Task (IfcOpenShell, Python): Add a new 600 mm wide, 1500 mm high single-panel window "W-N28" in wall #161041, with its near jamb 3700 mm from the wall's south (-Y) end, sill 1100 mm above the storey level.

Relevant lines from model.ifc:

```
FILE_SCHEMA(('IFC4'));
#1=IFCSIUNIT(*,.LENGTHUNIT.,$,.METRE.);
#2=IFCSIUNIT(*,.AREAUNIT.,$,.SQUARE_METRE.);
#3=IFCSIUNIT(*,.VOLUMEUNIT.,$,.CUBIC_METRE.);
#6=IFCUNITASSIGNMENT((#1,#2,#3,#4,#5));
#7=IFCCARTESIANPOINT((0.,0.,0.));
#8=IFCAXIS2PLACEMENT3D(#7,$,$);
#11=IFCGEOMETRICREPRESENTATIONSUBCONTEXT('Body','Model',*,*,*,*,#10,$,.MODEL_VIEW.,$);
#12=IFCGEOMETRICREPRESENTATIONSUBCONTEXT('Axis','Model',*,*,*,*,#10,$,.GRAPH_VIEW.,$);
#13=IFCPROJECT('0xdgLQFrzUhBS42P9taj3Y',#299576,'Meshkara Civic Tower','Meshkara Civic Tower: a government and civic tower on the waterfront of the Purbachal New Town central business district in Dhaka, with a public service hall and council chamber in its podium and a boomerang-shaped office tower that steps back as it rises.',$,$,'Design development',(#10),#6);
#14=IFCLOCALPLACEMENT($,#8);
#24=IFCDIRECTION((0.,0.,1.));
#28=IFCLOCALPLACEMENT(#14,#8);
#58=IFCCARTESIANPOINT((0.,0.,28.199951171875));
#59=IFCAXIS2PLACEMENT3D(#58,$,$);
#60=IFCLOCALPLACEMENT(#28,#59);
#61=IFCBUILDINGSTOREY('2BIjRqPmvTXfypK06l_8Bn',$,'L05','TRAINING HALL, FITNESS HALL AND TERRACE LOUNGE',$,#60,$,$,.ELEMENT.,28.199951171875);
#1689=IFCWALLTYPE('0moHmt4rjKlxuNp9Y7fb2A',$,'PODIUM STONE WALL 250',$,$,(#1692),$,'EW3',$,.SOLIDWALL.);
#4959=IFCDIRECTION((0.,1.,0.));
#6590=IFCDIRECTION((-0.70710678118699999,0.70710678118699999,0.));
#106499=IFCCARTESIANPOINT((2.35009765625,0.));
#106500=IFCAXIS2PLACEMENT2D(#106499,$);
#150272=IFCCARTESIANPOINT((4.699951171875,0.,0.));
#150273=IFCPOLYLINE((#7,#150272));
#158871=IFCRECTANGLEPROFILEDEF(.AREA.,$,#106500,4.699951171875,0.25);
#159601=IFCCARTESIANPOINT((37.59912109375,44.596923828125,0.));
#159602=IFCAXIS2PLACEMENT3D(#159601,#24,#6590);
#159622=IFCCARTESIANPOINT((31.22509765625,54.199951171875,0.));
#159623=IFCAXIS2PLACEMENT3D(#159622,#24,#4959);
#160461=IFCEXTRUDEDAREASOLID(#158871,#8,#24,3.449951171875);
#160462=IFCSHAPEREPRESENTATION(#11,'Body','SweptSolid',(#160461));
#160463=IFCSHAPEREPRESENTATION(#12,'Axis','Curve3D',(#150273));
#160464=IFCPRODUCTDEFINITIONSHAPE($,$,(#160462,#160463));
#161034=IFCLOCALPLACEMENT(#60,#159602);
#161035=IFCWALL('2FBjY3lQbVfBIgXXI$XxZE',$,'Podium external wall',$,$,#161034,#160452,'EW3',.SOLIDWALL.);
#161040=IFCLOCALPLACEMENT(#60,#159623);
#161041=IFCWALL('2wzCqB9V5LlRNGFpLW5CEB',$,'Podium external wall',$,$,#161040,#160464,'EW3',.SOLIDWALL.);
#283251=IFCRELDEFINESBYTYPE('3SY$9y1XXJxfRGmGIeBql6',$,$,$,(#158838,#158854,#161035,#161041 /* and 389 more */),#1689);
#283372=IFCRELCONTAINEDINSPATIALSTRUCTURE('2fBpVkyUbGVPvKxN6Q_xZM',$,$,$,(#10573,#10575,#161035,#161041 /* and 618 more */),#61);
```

```python
import numpy as np
import ifcopenshell
import ifcopenshell.api.feature
import ifcopenshell.api.geometry
import ifcopenshell.api.root
import ifcopenshell.api.spatial
import ifcopenshell.geom
import ifcopenshell.util.element
import ifcopenshell.util.placement
import ifcopenshell.util.representation
import ifcopenshell.util.shape
import ifcopenshell.util.unit

model = ifcopenshell.open("model.ifc")
unit_scale = ifcopenshell.util.unit.calculate_unit_scale(model)
settings = ifcopenshell.geom.settings()


def volume(element):
    """Net volume in cubic metres, openings subtracted."""
    shape = ifcopenshell.geom.create_shape(settings, element)
    return ifcopenshell.util.shape.get_volume(shape.geometry)


wall = model.by_guid("2wzCqB9V5LlRNGFpLW5CEB")
storey = ifcopenshell.util.element.get_container(wall, ifc_class="IfcBuildingStorey")
context = ifcopenshell.util.representation.get_context(model, "Model", "Body", "MODEL_VIEW")
before = volume(wall)

width, height, from_end, sill = 0.6, 1.5, 3.7, 1.1  # metres

# The wall runs along its own X axis, and the end named is its -X end.
wall_shape = ifcopenshell.geom.create_shape(settings, wall)
x, y, z = ifcopenshell.util.shape.get_vertices(wall_shape.geometry).T
start = x.min() + from_end
face, thickness = float(y.min()), float(y.max() - y.min())
wall_matrix = ifcopenshell.util.placement.get_local_placement(wall.ObjectPlacement)
level = ifcopenshell.util.placement.get_local_placement(storey.ObjectPlacement)[2, 3]


def in_wall(x, y):
    """Placement at x, y metres in the wall's axes, at sill height."""
    matrix = wall_matrix.copy()
    matrix[:, 3] = wall_matrix @ np.array([x / unit_scale, y / unit_scale, 0.0, 1.0])
    matrix[2, 3] = level + sill / unit_scale
    return matrix


# Opening: a box that overshoots both wall faces by 50 mm.
opening = ifcopenshell.api.root.create_entity(model, ifc_class="IfcOpeningElement", predefined_type="OPENING")
box = ifcopenshell.api.geometry.add_wall_representation(
    model, context=context, length=width, height=height, thickness=thickness + 0.1
)
ifcopenshell.api.geometry.assign_representation(model, product=opening, representation=box)
ifcopenshell.api.geometry.edit_object_placement(model, product=opening, matrix=in_wall(start, face - 0.05), is_si=False)
ifcopenshell.api.feature.add_feature(model, feature=opening, element=wall)

window = ifcopenshell.api.root.create_entity(model, ifc_class="IfcWindow", name="W-N28", predefined_type="WINDOW")
window.OverallWidth, window.OverallHeight = width / unit_scale, height / unit_scale
window.PartitioningType = "SINGLE_PANEL"
body = ifcopenshell.api.geometry.add_window_representation(
    model,
    context=context,
    overall_width=window.OverallWidth,
    overall_height=window.OverallHeight,
    partition_type="SINGLE_PANEL",
)
ifcopenshell.api.geometry.assign_representation(model, product=window, representation=body)
ifcopenshell.api.spatial.assign_container(model, products=[window], relating_structure=storey)
ifcopenshell.api.feature.add_filling(model, opening=opening, element=window)

# Centre the window in the wall's thickness.
ifcopenshell.api.geometry.edit_object_placement(model, product=window, matrix=in_wall(start, face), is_si=False)
window_shape = ifcopenshell.geom.create_shape(settings, window)
depth = ifcopenshell.util.shape.get_vertices(window_shape.geometry)[:, 1]
offset = face + thickness / 2 - (depth.min() + depth.max()) / 2
ifcopenshell.api.geometry.edit_object_placement(model, product=window, matrix=in_wall(start, offset), is_si=False)

after = volume(wall)

print(f"wall volume {before:.3f} -> {after:.3f} m3")

model.write("model_edited.ifc")
```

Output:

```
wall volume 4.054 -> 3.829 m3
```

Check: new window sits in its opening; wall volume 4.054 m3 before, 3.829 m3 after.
